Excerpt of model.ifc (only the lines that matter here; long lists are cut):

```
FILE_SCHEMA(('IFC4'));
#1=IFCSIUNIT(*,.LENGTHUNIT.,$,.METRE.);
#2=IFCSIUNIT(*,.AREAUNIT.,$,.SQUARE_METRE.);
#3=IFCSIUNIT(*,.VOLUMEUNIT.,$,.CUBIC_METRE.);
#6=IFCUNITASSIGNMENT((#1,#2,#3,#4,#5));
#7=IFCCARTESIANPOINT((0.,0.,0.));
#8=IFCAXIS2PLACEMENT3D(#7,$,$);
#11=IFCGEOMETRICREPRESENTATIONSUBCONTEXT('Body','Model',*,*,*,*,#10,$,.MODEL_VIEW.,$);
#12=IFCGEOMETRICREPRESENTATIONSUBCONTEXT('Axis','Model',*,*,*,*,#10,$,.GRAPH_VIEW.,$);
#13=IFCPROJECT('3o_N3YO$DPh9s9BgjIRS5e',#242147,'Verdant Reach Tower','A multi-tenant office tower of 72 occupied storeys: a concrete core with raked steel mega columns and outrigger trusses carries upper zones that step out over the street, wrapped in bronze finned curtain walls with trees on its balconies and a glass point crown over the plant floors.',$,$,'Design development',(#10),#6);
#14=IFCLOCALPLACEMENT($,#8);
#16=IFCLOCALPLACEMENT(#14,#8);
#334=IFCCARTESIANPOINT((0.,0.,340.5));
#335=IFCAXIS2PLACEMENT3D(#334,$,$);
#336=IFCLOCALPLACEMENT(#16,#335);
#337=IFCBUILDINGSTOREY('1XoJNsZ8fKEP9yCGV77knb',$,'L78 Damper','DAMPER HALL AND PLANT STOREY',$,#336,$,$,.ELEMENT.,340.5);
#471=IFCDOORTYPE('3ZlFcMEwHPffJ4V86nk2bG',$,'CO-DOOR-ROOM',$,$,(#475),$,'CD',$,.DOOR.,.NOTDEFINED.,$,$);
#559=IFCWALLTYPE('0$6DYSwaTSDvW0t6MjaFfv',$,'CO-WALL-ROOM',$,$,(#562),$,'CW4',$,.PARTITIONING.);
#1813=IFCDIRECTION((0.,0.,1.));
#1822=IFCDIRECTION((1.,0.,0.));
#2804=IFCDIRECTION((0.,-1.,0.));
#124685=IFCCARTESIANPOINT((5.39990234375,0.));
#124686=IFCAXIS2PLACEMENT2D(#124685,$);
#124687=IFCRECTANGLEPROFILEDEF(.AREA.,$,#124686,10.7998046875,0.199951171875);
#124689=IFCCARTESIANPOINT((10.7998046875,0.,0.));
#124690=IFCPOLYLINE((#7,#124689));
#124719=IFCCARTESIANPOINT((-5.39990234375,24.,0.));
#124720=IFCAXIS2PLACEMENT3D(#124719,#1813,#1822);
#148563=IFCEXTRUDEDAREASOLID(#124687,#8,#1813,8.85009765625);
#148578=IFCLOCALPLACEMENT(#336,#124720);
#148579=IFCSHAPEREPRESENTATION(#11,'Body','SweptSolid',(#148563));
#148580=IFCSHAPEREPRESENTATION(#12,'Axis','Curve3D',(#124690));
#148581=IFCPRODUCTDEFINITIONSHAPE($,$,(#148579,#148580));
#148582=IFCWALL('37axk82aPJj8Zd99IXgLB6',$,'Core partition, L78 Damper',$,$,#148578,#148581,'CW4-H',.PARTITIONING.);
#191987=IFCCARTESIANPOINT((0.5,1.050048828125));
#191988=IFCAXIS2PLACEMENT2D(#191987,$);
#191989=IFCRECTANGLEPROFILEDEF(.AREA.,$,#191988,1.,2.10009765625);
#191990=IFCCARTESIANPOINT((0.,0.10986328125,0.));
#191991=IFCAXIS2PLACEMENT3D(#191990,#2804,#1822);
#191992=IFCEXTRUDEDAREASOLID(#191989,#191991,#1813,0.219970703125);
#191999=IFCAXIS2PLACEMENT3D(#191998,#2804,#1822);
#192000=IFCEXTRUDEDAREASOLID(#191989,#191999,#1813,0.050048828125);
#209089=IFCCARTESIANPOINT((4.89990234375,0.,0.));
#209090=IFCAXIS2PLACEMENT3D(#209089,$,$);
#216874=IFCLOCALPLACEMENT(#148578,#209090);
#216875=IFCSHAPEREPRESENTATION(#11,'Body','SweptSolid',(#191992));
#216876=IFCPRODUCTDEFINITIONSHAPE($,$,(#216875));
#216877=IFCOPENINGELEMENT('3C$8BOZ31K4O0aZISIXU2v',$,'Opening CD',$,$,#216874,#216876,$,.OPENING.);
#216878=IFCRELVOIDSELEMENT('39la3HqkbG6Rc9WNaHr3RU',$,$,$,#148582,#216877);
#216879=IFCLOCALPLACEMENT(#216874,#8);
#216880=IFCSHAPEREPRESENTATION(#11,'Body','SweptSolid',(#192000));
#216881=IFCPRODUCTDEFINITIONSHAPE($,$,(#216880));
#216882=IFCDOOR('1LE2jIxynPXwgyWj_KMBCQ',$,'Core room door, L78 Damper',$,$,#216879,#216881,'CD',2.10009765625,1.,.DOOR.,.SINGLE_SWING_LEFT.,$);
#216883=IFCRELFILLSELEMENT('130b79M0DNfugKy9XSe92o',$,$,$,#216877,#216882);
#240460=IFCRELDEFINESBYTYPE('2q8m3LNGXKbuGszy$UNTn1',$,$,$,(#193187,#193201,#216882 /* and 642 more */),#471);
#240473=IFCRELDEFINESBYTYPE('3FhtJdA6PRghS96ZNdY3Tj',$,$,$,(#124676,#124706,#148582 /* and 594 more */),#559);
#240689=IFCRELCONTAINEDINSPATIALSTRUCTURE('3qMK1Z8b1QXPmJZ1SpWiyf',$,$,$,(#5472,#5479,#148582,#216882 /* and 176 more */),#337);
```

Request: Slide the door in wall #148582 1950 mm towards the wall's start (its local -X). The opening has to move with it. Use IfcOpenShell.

```python
import ifcopenshell
import ifcopenshell.api.geometry
import ifcopenshell.util.placement
import ifcopenshell.util.unit

model = ifcopenshell.open("model.ifc")
unit_scale = ifcopenshell.util.unit.calculate_unit_scale(model)

door = model.by_guid("1LE2jIxynPXwgyWj_KMBCQ")
opening = door.FillsVoids[0].RelatingOpeningElement
wall = opening.VoidsElements[0].RelatingBuildingElement

wall_matrix = ifcopenshell.util.placement.get_local_placement(wall.ObjectPlacement)
shift = wall_matrix[:3, 0] * -1.95 / unit_scale
before = ifcopenshell.util.placement.get_local_placement(door.ObjectPlacement)[:3, 3].copy()

# The door is placed relative to its opening, so it follows when the opening moves.
matrix = ifcopenshell.util.placement.get_local_placement(opening.ObjectPlacement)
matrix[:3, 3] += shift
ifcopenshell.api.geometry.edit_object_placement(
    model, product=opening, matrix=matrix, is_si=False, should_transform_children=True
)

after = ifcopenshell.util.placement.get_local_placement(door.ObjectPlacement)[:3, 3]
print("door moved by", (after - before).round(3) + 0.0)

model.write("model_edited.ifc")
```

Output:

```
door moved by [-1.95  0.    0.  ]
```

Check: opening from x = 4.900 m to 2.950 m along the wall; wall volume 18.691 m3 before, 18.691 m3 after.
